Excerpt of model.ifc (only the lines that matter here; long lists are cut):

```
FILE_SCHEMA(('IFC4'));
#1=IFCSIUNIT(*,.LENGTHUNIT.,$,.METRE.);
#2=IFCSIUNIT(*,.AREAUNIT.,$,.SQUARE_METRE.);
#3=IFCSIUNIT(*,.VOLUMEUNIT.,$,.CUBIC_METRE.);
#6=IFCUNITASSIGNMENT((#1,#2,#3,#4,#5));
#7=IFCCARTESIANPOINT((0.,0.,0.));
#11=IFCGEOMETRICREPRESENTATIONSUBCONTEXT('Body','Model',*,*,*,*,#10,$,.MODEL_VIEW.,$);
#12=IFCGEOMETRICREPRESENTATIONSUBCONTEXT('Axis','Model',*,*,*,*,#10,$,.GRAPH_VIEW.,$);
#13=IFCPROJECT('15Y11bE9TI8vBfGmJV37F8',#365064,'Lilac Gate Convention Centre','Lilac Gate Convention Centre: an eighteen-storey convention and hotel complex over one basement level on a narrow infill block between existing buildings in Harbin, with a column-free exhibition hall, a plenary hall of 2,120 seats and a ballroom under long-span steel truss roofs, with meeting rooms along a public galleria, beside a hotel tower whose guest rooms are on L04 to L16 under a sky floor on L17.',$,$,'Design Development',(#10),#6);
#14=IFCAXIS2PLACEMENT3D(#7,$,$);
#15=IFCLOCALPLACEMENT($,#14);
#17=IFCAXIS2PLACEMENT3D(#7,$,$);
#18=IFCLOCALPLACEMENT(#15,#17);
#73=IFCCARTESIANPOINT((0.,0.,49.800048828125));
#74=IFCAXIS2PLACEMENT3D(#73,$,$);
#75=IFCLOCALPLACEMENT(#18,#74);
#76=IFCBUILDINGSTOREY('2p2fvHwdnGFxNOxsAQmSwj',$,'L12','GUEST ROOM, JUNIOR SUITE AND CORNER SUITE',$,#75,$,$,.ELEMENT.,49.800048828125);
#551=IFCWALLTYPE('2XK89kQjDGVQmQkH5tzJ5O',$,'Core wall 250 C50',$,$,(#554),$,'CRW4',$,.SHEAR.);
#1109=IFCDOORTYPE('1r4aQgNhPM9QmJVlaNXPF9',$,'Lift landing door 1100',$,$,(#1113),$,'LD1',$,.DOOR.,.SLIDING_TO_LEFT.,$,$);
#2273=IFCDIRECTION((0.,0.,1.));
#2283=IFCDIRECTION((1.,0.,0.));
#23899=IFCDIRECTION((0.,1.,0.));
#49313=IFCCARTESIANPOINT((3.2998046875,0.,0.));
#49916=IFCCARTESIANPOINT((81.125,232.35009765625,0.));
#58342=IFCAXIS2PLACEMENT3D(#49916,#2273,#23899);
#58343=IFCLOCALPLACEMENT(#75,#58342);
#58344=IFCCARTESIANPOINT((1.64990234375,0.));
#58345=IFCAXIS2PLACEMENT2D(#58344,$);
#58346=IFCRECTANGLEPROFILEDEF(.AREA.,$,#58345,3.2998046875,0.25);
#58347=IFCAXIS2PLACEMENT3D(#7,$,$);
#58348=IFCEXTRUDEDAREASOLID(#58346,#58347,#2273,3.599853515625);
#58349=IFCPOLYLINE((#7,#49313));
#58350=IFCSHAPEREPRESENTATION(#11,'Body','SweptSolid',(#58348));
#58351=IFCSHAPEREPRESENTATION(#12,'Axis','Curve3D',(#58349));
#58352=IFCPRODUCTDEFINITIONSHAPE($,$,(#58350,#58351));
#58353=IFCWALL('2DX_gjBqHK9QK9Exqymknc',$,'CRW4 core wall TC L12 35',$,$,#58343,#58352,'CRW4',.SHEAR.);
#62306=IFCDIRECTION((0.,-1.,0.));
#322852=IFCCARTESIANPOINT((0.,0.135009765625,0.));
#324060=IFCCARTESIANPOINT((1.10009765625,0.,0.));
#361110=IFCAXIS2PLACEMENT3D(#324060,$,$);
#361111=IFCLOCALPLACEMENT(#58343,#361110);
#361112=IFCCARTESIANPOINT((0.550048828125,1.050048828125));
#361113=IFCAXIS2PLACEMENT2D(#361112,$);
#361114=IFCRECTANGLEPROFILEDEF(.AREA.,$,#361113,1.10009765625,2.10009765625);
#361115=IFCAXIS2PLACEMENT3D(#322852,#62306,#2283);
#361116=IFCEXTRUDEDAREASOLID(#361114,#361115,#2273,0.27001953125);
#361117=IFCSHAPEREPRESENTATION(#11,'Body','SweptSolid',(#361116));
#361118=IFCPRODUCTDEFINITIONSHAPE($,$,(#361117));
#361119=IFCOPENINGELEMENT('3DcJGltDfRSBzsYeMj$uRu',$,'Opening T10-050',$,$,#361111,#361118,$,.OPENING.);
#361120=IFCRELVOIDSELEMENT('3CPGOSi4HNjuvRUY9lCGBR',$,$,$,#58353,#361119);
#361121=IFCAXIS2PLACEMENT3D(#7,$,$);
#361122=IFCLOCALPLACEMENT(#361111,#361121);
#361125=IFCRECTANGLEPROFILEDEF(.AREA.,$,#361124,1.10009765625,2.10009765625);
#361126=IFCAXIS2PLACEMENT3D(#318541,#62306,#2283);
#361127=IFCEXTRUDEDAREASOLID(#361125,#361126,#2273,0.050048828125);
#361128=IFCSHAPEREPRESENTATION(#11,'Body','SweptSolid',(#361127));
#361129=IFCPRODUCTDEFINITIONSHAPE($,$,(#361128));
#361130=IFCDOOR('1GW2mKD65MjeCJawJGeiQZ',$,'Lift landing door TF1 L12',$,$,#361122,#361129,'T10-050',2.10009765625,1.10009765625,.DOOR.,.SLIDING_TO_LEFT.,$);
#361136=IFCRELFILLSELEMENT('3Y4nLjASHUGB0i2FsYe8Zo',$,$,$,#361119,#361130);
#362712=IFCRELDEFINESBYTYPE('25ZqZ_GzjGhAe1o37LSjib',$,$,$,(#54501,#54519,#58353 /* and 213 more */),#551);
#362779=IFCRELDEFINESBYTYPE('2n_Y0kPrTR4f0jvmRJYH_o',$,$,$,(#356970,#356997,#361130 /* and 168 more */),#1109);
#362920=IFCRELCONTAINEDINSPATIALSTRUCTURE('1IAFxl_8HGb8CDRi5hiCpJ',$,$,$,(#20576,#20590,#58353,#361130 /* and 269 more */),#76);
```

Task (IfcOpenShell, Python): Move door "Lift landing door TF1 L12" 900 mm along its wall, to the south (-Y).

```python
import ifcopenshell
import ifcopenshell.api.geometry
import ifcopenshell.util.placement

model = ifcopenshell.open("model.ifc")

door = model.by_guid("1GW2mKD65MjeCJawJGeiQZ")
opening = door.FillsVoids[0].RelatingOpeningElement
wall = opening.VoidsElements[0].RelatingBuildingElement

wall_matrix = ifcopenshell.util.placement.get_local_placement(wall.ObjectPlacement)
shift = wall_matrix[:3, 0] * -0.9
before = ifcopenshell.util.placement.get_local_placement(door.ObjectPlacement)[:3, 3].copy()

# The door is placed relative to its opening, so it follows when the opening moves.
matrix = ifcopenshell.util.placement.get_local_placement(opening.ObjectPlacement)
matrix[:3, 3] += shift
ifcopenshell.api.geometry.edit_object_placement(
    model, product=opening, matrix=matrix, is_si=False, should_transform_children=True
)

after = ifcopenshell.util.placement.get_local_placement(door.ObjectPlacement)[:3, 3]
print("door moved by", (after - before).round(3) + 0.0)

model.write("model_updated.ifc")
```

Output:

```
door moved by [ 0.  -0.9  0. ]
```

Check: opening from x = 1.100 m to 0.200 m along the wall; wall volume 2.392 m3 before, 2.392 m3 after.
